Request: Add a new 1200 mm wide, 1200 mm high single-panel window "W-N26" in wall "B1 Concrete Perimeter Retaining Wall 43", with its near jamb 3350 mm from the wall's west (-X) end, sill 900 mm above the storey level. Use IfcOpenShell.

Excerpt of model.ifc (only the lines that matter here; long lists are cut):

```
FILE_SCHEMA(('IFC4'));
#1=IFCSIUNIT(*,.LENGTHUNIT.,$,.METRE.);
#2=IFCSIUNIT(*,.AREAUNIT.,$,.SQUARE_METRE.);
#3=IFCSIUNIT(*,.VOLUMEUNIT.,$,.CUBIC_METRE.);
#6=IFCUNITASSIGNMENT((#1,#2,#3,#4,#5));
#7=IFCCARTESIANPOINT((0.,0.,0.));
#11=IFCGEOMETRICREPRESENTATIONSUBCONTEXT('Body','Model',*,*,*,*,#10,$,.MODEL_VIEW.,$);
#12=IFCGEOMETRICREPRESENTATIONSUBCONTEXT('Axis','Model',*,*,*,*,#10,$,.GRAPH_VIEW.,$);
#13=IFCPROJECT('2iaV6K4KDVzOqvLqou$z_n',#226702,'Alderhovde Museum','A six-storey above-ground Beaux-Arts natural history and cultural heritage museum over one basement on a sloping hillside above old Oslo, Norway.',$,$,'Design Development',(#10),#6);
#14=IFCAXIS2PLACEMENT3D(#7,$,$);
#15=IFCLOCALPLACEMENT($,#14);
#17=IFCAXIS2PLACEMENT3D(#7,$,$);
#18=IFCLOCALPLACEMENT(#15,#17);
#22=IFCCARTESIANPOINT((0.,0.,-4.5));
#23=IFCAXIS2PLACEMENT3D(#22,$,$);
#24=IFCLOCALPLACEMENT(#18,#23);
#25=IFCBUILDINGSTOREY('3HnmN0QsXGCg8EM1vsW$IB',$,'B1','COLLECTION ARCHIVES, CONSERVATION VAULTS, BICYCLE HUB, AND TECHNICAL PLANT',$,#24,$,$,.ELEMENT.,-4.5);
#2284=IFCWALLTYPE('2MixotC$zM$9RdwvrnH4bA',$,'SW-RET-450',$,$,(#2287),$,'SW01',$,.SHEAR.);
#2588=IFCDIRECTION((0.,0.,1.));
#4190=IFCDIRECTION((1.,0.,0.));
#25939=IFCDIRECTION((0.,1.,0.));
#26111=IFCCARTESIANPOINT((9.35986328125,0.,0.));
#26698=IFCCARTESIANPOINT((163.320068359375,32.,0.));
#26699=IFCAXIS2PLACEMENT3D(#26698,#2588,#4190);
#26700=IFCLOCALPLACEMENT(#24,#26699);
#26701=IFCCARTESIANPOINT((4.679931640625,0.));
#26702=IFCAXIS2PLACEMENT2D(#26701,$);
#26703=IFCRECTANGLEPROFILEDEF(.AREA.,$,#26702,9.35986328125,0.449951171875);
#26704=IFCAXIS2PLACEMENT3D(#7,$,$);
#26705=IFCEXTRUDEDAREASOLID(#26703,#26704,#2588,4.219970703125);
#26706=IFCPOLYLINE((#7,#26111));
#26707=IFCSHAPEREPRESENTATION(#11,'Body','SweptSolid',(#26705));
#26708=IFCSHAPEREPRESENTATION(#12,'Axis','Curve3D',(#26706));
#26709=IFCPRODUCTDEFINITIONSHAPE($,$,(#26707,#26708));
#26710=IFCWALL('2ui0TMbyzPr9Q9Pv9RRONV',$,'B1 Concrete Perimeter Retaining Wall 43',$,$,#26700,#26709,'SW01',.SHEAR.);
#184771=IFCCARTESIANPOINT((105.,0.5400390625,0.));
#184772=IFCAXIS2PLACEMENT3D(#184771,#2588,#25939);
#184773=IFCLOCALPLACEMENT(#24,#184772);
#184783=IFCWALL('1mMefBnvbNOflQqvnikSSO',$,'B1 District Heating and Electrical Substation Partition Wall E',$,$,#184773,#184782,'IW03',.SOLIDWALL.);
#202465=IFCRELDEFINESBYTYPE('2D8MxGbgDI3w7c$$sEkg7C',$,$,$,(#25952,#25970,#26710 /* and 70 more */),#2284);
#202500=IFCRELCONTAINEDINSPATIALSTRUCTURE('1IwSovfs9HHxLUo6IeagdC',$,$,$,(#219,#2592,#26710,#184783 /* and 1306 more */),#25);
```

```python
import numpy as np
import ifcopenshell
import ifcopenshell.api.feature
import ifcopenshell.api.geometry
import ifcopenshell.api.root
import ifcopenshell.api.spatial
import ifcopenshell.geom
import ifcopenshell.util.element
import ifcopenshell.util.placement
import ifcopenshell.util.representation
import ifcopenshell.util.shape
import ifcopenshell.util.unit

model = ifcopenshell.open("model.ifc")
unit_scale = ifcopenshell.util.unit.calculate_unit_scale(model)
settings = ifcopenshell.geom.settings()


def volume(element):
    """Net volume in cubic metres, openings subtracted."""
    shape = ifcopenshell.geom.create_shape(settings, element)
    return ifcopenshell.util.shape.get_volume(shape.geometry)


wall = model.by_guid("2ui0TMbyzPr9Q9Pv9RRONV")
storey = ifcopenshell.util.element.get_container(wall, ifc_class="IfcBuildingStorey")
context = ifcopenshell.util.representation.get_context(model, "Model", "Body", "MODEL_VIEW")
before = volume(wall)

width, height, from_end, sill = 1.2, 1.2, 3.35, 0.9  # metres

# The wall runs along its own X axis, and the end named is its -X end.
wall_shape = ifcopenshell.geom.create_shape(settings, wall)
x, y, z = ifcopenshell.util.shape.get_vertices(wall_shape.geometry).T
start = x.min() + from_end
face, thickness = float(y.min()), float(y.max() - y.min())
wall_matrix = ifcopenshell.util.placement.get_local_placement(wall.ObjectPlacement)
level = ifcopenshell.util.placement.get_local_placement(storey.ObjectPlacement)[2, 3]


def in_wall(x, y):
    """Placement at x, y metres in the wall's axes, at sill height."""
    matrix = wall_matrix.copy()
    matrix[:, 3] = wall_matrix @ np.array([x / unit_scale, y / unit_scale, 0.0, 1.0])
    matrix[2, 3] = level + sill / unit_scale
    return matrix


# Opening: a box that overshoots both wall faces by 50 mm.
opening = ifcopenshell.api.root.create_entity(model, ifc_class="IfcOpeningElement", predefined_type="OPENING")
box = ifcopenshell.api.geometry.add_wall_representation(
    model, context=context, length=width, height=height, thickness=thickness + 0.1
)
ifcopenshell.api.geometry.assign_representation(model, product=opening, representation=box)
ifcopenshell.api.geometry.edit_object_placement(model, product=opening, matrix=in_wall(start, face - 0.05), is_si=False)
ifcopenshell.api.feature.add_feature(model, feature=opening, element=wall)

window = ifcopenshell.api.root.create_entity(model, ifc_class="IfcWindow", name="W-N26", predefined_type="WINDOW")
window.OverallWidth, window.OverallHeight = width / unit_scale, height / unit_scale
window.PartitioningType = "SINGLE_PANEL"
body = ifcopenshell.api.geometry.add_window_representation(
    model,
    context=context,
    overall_width=window.OverallWidth,
    overall_height=window.OverallHeight,
    partition_type="SINGLE_PANEL",
)
ifcopenshell.api.geometry.assign_representation(model, product=window, representation=body)
ifcopenshell.api.spatial.assign_container(model, products=[window], relating_structure=storey)
ifcopenshell.api.feature.add_filling(model, opening=opening, element=window)

# Centre the window in the wall's thickness.
ifcopenshell.api.geometry.edit_object_placement(model, product=window, matrix=in_wall(start, face), is_si=False)
window_shape = ifcopenshell.geom.create_shape(settings, window)
depth = ifcopenshell.util.shape.get_vertices(window_shape.geometry)[:, 1]
offset = face + thickness / 2 - (depth.min() + depth.max()) / 2
ifcopenshell.api.geometry.edit_object_placement(model, product=window, matrix=in_wall(start, offset), is_si=False)

after = volume(wall)

print(f"wall volume {before:.3f} -> {after:.3f} m3")

model.write("model_updated.ifc")
```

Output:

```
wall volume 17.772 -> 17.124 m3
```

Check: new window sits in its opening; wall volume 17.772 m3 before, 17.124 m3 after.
